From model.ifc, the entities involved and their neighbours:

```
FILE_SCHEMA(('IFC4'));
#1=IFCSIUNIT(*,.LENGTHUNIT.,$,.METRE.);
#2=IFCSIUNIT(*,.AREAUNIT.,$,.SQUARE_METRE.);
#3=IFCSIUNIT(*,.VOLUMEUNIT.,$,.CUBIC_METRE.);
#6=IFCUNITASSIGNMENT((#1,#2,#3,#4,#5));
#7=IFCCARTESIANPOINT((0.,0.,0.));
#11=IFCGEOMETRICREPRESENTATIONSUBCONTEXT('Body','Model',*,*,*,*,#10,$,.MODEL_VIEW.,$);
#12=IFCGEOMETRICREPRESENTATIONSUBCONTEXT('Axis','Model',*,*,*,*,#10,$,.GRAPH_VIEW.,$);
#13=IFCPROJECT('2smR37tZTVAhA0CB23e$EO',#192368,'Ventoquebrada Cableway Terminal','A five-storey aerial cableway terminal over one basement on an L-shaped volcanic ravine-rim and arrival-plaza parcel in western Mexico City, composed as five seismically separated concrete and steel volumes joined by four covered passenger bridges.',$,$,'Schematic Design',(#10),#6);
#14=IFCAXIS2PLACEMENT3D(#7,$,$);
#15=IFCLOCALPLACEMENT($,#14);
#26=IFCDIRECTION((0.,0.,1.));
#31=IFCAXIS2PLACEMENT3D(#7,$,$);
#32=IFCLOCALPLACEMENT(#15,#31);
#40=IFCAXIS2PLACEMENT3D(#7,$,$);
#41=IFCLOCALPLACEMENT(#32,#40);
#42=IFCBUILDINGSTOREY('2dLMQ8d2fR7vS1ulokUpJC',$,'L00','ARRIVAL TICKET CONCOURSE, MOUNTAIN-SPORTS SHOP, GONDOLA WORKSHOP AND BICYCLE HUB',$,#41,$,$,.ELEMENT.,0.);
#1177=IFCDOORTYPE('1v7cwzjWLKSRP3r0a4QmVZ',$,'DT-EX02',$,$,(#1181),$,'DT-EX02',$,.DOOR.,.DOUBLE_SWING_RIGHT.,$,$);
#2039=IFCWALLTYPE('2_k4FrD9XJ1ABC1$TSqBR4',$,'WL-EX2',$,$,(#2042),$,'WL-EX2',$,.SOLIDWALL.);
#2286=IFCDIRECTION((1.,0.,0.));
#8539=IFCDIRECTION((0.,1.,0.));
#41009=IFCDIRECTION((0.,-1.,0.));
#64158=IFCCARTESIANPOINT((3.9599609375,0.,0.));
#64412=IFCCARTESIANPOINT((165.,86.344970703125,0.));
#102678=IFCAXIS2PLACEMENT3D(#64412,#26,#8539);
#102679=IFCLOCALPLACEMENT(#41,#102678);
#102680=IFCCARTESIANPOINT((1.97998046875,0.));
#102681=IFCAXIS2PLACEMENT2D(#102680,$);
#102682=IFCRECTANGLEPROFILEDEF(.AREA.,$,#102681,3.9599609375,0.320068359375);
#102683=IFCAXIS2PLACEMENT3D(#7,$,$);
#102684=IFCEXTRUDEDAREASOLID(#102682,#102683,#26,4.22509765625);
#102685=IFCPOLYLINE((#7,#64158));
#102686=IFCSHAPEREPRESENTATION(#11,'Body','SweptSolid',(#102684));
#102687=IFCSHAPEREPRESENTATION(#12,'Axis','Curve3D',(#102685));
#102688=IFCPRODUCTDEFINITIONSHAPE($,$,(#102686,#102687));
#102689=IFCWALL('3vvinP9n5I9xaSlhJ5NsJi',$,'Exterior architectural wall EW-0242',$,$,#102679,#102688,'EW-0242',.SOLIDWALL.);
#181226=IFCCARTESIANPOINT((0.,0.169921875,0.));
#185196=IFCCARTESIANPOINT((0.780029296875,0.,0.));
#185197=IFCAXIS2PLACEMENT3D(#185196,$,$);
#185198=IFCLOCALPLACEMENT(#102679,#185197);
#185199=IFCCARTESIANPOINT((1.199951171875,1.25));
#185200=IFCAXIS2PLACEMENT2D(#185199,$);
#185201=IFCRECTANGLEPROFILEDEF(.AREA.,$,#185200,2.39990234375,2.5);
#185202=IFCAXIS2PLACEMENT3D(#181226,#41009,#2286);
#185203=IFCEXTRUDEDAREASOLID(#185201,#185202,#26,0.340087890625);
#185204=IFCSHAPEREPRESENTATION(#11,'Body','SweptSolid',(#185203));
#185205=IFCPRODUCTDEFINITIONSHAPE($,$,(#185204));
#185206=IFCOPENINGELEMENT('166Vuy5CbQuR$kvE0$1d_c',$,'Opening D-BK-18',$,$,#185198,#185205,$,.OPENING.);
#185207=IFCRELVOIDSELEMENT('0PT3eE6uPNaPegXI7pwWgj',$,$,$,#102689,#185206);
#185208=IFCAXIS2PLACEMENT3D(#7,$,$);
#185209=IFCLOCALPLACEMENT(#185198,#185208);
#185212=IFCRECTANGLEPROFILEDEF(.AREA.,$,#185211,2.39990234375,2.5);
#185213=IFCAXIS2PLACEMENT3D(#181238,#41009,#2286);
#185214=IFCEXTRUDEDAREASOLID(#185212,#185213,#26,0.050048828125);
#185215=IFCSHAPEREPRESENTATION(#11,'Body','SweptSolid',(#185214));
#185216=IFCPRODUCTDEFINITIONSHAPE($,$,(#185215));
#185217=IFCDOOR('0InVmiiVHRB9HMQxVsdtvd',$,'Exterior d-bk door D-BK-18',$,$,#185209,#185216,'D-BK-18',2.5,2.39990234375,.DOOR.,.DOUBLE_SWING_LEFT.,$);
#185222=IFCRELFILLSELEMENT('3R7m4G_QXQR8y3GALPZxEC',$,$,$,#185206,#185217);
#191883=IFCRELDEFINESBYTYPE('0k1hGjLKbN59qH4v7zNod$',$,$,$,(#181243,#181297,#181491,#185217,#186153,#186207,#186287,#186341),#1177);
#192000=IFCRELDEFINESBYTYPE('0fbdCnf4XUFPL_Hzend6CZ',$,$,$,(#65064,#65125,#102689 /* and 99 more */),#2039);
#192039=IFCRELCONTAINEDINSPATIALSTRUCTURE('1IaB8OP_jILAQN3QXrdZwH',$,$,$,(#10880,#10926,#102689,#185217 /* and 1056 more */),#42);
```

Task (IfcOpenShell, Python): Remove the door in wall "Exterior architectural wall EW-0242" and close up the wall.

```python
import ifcopenshell
import ifcopenshell.api.feature
import ifcopenshell.api.root
import ifcopenshell.geom
import ifcopenshell.util.shape

model = ifcopenshell.open("model.ifc")
settings = ifcopenshell.geom.settings()


def volume(element):
    """Net volume in cubic metres, openings subtracted."""
    shape = ifcopenshell.geom.create_shape(settings, element)
    return ifcopenshell.util.shape.get_volume(shape.geometry)


door = model.by_guid("0InVmiiVHRB9HMQxVsdtvd")
opening = door.FillsVoids[0].RelatingOpeningElement
wall = opening.VoidsElements[0].RelatingBuildingElement
before = volume(wall)

ifcopenshell.api.root.remove_product(model, product=door)
ifcopenshell.api.feature.remove_feature(model, feature=opening)

after = volume(wall)

print(f"wall volume {before:.3f} -> {after:.3f} m3")

model.write("model-out.ifc")
```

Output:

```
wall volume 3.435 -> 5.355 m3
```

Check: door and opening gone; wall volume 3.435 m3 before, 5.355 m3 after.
